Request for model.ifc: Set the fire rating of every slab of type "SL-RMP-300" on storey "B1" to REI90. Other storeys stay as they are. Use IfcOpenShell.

First a look at what the model holds.

```python
import ifcopenshell
import ifcopenshell.util.element

model = ifcopenshell.open("model.ifc")
print(model.schema)
storey = next(s for s in model.by_type("IfcBuildingStorey") if s.Name == "B1")
slabs = [e for e in ifcopenshell.util.element.get_decomposition(storey) if e.is_a("IfcSlab")]
seen = {}
for e in slabs:
    element_type = ifcopenshell.util.element.get_type(e)
    key = (element_type.Name if element_type != e and element_type else None, ifcopenshell.util.element.get_pset(e, "Pset_SlabCommon", "FireRating"))
    seen[key] = seen.get(key, 0) + 1
for (name, value), count in sorted(seen.items(), key=str):
    print(count, "x", name, "|", value)
```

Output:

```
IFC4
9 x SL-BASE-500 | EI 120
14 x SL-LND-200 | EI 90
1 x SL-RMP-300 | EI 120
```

```python
import ifcopenshell
import ifcopenshell.api.pset
import ifcopenshell.util.element

model = ifcopenshell.open("model.ifc")

storey = next(s for s in model.by_type("IfcBuildingStorey") if s.Name == "B1")
slabs = [e for e in ifcopenshell.util.element.get_decomposition(storey) if e.is_a("IfcSlab")]

count = 0
for e in slabs:
    element_type = ifcopenshell.util.element.get_type(e)
    if element_type in (None, e) or element_type.Name != "SL-RMP-300":
        continue
    # add_pset returns the element's existing set when there is one.
    pset = ifcopenshell.api.pset.add_pset(model, product=e, name="Pset_SlabCommon")
    ifcopenshell.api.pset.edit_pset(model, pset=pset, properties={"FireRating": "REI90"})
    count += 1

print(count, "slabs updated")

model.write("model_rev.ifc")
```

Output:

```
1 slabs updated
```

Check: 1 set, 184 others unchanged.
